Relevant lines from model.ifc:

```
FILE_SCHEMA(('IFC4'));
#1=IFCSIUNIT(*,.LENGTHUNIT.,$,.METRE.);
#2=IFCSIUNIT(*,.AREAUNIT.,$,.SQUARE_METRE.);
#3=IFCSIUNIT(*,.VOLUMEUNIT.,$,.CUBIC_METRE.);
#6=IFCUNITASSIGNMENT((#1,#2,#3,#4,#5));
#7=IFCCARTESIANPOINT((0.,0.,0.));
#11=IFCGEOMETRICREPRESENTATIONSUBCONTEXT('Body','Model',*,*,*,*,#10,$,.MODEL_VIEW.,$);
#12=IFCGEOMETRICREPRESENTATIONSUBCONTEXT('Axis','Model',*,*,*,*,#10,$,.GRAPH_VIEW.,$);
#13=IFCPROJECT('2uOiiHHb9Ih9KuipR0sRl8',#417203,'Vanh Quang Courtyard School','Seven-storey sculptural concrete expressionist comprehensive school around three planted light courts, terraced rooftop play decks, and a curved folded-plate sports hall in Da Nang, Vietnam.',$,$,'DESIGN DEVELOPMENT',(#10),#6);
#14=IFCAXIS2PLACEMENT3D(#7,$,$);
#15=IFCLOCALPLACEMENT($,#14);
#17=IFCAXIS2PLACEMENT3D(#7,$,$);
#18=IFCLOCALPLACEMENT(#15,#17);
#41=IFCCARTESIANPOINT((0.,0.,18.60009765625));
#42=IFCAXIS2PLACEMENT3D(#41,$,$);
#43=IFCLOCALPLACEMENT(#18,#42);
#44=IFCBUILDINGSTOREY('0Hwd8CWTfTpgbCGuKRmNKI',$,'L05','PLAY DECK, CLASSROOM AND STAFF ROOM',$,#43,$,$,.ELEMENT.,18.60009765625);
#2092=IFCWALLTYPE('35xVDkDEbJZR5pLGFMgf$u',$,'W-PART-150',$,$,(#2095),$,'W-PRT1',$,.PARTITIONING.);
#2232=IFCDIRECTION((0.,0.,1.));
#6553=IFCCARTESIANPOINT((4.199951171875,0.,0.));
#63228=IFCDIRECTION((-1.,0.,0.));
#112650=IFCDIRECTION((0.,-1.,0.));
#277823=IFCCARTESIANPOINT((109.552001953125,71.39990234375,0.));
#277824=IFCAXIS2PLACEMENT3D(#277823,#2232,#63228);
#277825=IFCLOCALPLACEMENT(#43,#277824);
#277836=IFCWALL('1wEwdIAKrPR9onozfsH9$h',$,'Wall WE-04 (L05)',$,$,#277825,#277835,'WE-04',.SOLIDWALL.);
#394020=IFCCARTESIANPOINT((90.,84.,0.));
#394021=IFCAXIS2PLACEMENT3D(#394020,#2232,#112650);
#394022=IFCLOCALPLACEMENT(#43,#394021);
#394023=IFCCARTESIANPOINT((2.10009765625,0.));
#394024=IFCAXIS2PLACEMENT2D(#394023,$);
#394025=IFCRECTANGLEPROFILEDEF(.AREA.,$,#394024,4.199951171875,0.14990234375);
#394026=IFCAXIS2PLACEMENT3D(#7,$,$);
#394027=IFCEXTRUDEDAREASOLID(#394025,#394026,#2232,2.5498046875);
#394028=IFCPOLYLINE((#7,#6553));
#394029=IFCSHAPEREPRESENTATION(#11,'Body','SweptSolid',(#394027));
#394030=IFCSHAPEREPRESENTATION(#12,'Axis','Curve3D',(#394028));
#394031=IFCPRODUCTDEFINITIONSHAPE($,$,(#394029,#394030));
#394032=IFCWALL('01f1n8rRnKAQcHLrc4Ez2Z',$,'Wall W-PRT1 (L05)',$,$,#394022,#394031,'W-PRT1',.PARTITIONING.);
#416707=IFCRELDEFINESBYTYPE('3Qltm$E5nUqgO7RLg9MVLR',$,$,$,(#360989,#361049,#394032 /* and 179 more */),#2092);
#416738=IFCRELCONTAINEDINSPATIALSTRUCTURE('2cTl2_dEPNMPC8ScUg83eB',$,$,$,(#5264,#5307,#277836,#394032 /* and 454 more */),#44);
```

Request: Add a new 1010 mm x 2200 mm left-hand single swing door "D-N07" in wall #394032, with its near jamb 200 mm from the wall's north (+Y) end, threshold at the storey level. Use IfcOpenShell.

```python
import numpy as np
import ifcopenshell
import ifcopenshell.api.feature
import ifcopenshell.api.geometry
import ifcopenshell.api.root
import ifcopenshell.api.spatial
import ifcopenshell.geom
import ifcopenshell.util.element
import ifcopenshell.util.placement
import ifcopenshell.util.representation
import ifcopenshell.util.shape
import ifcopenshell.util.unit

model = ifcopenshell.open("model.ifc")
unit_scale = ifcopenshell.util.unit.calculate_unit_scale(model)
settings = ifcopenshell.geom.settings()


def volume(element):
    """Net volume in cubic metres, openings subtracted."""
    shape = ifcopenshell.geom.create_shape(settings, element)
    return ifcopenshell.util.shape.get_volume(shape.geometry)


wall = model.by_id(394032)
storey = ifcopenshell.util.element.get_container(wall, ifc_class="IfcBuildingStorey")
context = ifcopenshell.util.representation.get_context(model, "Model", "Body", "MODEL_VIEW")
before = volume(wall)

width, height, from_end, sill = 1.01, 2.2, 0.2, 0.0  # metres

# The wall runs along its own X axis, and the end named is its -X end.
wall_shape = ifcopenshell.geom.create_shape(settings, wall)
x, y, z = ifcopenshell.util.shape.get_vertices(wall_shape.geometry).T
start = x.min() + from_end
face, thickness = float(y.min()), float(y.max() - y.min())
wall_matrix = ifcopenshell.util.placement.get_local_placement(wall.ObjectPlacement)
level = ifcopenshell.util.placement.get_local_placement(storey.ObjectPlacement)[2, 3]


def in_wall(x, y):
    """Placement at x, y metres in the wall's axes, at sill height."""
    matrix = wall_matrix.copy()
    matrix[:, 3] = wall_matrix @ np.array([x / unit_scale, y / unit_scale, 0.0, 1.0])
    matrix[2, 3] = level + sill / unit_scale
    return matrix


# Opening: a box that overshoots both wall faces by 50 mm.
opening = ifcopenshell.api.root.create_entity(model, ifc_class="IfcOpeningElement", predefined_type="OPENING")
box = ifcopenshell.api.geometry.add_wall_representation(
    model, context=context, length=width, height=height, thickness=thickness + 0.1
)
ifcopenshell.api.geometry.assign_representation(model, product=opening, representation=box)
ifcopenshell.api.geometry.edit_object_placement(model, product=opening, matrix=in_wall(start, face - 0.05), is_si=False)
ifcopenshell.api.feature.add_feature(model, feature=opening, element=wall)

door = ifcopenshell.api.root.create_entity(model, ifc_class="IfcDoor", name="D-N07", predefined_type="DOOR")
door.OverallWidth, door.OverallHeight = width / unit_scale, height / unit_scale
door.OperationType = "SINGLE_SWING_LEFT"
body = ifcopenshell.api.geometry.add_door_representation(
    model,
    context=context,
    overall_width=door.OverallWidth,
    overall_height=door.OverallHeight,
    operation_type="SINGLE_SWING_LEFT",
    lining_properties={"LiningDepth": thickness / unit_scale, "ThresholdDepth": thickness / unit_scale},
)
ifcopenshell.api.geometry.assign_representation(model, product=door, representation=body)
ifcopenshell.api.spatial.assign_container(model, products=[door], relating_structure=storey)
ifcopenshell.api.feature.add_filling(model, opening=opening, element=door)

# The lining spans the wall, so the door starts at the wall face.
ifcopenshell.api.geometry.edit_object_placement(model, product=door, matrix=in_wall(start, face), is_si=False)

after = volume(wall)

print(f"wall volume {before:.3f} -> {after:.3f} m3")

model.write("model-out.ifc")
```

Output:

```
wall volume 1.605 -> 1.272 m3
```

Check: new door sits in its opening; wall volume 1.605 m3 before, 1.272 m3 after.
